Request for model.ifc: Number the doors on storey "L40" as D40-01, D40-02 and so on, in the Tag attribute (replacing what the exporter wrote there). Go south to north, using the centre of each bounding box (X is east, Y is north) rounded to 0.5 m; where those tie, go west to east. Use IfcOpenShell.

First a look at what the model holds.

```python
import ifcopenshell
import ifcopenshell.util.element
import ifcopenshell.util.placement

model = ifcopenshell.open("model.ifc")
print(model.schema)
storey = next(s for s in model.by_type("IfcBuildingStorey") if s.Name == "L40")
doors = [e for e in ifcopenshell.util.element.get_decomposition(storey) if e.is_a("IfcDoor")]
for e in sorted(doors, key=lambda e: e.id()):
    origin = ifcopenshell.util.placement.get_local_placement(e.ObjectPlacement)[:3, 3]
    print(e.id(), e.Tag, e.Name, origin.round(2) + 0.0, sep=" | ")
```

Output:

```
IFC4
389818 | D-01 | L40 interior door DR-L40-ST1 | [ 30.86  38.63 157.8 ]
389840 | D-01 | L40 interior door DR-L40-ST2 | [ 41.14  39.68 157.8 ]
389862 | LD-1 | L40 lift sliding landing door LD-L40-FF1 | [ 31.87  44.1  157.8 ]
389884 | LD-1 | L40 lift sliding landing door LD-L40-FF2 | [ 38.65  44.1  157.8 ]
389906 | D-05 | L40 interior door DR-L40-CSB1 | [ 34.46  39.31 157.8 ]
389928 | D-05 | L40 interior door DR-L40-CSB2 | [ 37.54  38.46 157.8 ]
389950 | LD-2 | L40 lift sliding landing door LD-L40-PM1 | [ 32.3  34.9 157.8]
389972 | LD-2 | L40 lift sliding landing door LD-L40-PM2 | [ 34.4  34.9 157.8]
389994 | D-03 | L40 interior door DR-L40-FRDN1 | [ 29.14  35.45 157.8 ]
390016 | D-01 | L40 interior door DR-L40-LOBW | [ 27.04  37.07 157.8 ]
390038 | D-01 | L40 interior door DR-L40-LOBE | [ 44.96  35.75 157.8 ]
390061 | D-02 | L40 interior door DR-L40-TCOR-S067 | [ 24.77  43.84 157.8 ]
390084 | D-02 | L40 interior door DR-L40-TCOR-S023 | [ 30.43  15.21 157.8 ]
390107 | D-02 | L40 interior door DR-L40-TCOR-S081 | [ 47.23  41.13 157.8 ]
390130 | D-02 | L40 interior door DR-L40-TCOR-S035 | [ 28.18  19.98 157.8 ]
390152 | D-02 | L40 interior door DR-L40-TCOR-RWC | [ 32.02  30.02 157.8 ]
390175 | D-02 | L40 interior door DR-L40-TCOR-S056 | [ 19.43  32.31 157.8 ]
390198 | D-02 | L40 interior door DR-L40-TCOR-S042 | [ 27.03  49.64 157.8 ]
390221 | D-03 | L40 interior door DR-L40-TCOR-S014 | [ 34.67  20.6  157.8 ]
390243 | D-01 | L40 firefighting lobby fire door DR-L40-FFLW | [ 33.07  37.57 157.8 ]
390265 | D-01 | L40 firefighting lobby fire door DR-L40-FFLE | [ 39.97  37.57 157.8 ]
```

```python
import ifcopenshell
import ifcopenshell.geom
import ifcopenshell.util.element
import ifcopenshell.util.shape

model = ifcopenshell.open("model.ifc")
settings = ifcopenshell.geom.settings()
settings.set("use-world-coords", True)


def centre(element):
    shape = ifcopenshell.geom.create_shape(settings, element)
    return ifcopenshell.util.shape.get_bbox_centroid(shape.geometry)


storey = next(s for s in model.by_type("IfcBuildingStorey") if s.Name == "L40")
doors = [e for e in ifcopenshell.util.element.get_decomposition(storey) if e.is_a("IfcDoor")]

# Insertion points can sit at a corner or the storey origin, so sort by the geometry (in metres).
centres = {e: centre(e) for e in doors}
doors.sort(key=lambda e: (round(centres[e][1] / 0.5), centres[e][0]))

for i, e in enumerate(doors, start=1):
    number = f"D40-{i:02d}"
    e.Tag = number
    print(e.id(), number)

model.write("model_v2.ifc")
```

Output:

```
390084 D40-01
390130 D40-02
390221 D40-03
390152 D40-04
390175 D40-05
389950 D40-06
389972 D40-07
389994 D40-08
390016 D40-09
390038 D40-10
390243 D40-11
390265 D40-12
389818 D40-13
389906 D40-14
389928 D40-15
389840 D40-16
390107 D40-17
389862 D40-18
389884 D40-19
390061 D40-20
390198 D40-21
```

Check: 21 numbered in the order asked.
